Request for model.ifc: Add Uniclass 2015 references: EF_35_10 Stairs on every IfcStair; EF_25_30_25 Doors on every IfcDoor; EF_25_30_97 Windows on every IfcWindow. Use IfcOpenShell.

First a look at what the model holds.

```python
import ifcopenshell

model = ifcopenshell.open("model.ifc")
print(model.schema)
print("classifications:", [c.Name for c in model.by_type("IfcClassification")])
for ifc_class in ("IfcDoor", "IfcRoof", "IfcStair", "IfcWall", "IfcWindow"):
    print(ifc_class, len(model.by_type(ifc_class)))
```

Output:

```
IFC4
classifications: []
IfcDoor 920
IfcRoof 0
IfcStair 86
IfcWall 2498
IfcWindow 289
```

```python
import ifcopenshell
import ifcopenshell.api.classification

model = ifcopenshell.open("model.ifc")

system = ifcopenshell.api.classification.add_classification(model, classification="Uniclass 2015")

codes = {
    "IfcStair": ("EF_35_10", "Stairs"),
    "IfcDoor": ("EF_25_30_25", "Doors"),
    "IfcWindow": ("EF_25_30_97", "Windows"),
}
for ifc_class, (code, name) in codes.items():
    products = model.by_type(ifc_class)
    ifcopenshell.api.classification.add_reference(
        model, products=products, classification=system, identification=code, name=name
    )
    print(code, len(products))

model.write("model_edited.ifc")
```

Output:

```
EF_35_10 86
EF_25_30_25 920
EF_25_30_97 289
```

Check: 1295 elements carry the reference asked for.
